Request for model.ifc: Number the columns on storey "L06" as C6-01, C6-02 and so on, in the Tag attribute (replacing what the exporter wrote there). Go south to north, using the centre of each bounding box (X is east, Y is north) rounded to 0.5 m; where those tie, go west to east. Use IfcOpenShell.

First a look at what the model holds.

```python
import ifcopenshell
import ifcopenshell.util.element
import ifcopenshell.util.placement

model = ifcopenshell.open("model.ifc")
print(model.schema)
storey = next(s for s in model.by_type("IfcBuildingStorey") if s.Name == "L06")
columns = [e for e in ifcopenshell.util.element.get_decomposition(storey) if e.is_a("IfcColumn")]
for e in sorted(columns, key=lambda e: e.id()):
    origin = ifcopenshell.util.placement.get_local_placement(e.ObjectPlacement)[:3, 3]
    print(e.id(), e.Tag, e.Name, origin.round(2) + 0.0, sep=" | ")
```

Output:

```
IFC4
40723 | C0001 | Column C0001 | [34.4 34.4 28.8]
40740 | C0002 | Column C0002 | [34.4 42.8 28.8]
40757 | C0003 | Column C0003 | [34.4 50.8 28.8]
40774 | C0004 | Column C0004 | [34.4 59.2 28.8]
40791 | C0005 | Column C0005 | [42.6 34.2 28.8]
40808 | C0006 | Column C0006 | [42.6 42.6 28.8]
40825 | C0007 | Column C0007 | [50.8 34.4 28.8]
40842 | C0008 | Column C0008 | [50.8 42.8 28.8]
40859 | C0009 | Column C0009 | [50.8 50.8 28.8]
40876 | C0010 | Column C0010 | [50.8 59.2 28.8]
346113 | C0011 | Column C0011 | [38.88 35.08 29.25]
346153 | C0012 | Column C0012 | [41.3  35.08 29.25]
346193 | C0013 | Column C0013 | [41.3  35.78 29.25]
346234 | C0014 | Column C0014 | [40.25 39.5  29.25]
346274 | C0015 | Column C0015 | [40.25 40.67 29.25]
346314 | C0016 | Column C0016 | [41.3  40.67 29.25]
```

```python
import ifcopenshell
import ifcopenshell.geom
import ifcopenshell.util.element
import ifcopenshell.util.shape

model = ifcopenshell.open("model.ifc")
settings = ifcopenshell.geom.settings()
settings.set("use-world-coords", True)


def centre(element):
    shape = ifcopenshell.geom.create_shape(settings, element)
    return ifcopenshell.util.shape.get_bbox_centroid(shape.geometry)


storey = next(s for s in model.by_type("IfcBuildingStorey") if s.Name == "L06")
columns = [e for e in ifcopenshell.util.element.get_decomposition(storey) if e.is_a("IfcColumn")]

# Insertion points can sit at a corner or the storey origin, so sort by the geometry (in metres).
centres = {e: centre(e) for e in columns}
columns.sort(key=lambda e: (round(centres[e][1] / 0.5), centres[e][0]))

for i, e in enumerate(columns, start=1):
    number = f"C6-{i:02d}"
    e.Tag = number
    print(e.id(), number)

model.write("model_v2.ifc")
```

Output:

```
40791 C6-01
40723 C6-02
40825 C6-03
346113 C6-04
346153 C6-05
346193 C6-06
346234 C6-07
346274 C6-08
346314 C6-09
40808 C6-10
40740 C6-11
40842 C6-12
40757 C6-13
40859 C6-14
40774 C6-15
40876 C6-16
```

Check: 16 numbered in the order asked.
